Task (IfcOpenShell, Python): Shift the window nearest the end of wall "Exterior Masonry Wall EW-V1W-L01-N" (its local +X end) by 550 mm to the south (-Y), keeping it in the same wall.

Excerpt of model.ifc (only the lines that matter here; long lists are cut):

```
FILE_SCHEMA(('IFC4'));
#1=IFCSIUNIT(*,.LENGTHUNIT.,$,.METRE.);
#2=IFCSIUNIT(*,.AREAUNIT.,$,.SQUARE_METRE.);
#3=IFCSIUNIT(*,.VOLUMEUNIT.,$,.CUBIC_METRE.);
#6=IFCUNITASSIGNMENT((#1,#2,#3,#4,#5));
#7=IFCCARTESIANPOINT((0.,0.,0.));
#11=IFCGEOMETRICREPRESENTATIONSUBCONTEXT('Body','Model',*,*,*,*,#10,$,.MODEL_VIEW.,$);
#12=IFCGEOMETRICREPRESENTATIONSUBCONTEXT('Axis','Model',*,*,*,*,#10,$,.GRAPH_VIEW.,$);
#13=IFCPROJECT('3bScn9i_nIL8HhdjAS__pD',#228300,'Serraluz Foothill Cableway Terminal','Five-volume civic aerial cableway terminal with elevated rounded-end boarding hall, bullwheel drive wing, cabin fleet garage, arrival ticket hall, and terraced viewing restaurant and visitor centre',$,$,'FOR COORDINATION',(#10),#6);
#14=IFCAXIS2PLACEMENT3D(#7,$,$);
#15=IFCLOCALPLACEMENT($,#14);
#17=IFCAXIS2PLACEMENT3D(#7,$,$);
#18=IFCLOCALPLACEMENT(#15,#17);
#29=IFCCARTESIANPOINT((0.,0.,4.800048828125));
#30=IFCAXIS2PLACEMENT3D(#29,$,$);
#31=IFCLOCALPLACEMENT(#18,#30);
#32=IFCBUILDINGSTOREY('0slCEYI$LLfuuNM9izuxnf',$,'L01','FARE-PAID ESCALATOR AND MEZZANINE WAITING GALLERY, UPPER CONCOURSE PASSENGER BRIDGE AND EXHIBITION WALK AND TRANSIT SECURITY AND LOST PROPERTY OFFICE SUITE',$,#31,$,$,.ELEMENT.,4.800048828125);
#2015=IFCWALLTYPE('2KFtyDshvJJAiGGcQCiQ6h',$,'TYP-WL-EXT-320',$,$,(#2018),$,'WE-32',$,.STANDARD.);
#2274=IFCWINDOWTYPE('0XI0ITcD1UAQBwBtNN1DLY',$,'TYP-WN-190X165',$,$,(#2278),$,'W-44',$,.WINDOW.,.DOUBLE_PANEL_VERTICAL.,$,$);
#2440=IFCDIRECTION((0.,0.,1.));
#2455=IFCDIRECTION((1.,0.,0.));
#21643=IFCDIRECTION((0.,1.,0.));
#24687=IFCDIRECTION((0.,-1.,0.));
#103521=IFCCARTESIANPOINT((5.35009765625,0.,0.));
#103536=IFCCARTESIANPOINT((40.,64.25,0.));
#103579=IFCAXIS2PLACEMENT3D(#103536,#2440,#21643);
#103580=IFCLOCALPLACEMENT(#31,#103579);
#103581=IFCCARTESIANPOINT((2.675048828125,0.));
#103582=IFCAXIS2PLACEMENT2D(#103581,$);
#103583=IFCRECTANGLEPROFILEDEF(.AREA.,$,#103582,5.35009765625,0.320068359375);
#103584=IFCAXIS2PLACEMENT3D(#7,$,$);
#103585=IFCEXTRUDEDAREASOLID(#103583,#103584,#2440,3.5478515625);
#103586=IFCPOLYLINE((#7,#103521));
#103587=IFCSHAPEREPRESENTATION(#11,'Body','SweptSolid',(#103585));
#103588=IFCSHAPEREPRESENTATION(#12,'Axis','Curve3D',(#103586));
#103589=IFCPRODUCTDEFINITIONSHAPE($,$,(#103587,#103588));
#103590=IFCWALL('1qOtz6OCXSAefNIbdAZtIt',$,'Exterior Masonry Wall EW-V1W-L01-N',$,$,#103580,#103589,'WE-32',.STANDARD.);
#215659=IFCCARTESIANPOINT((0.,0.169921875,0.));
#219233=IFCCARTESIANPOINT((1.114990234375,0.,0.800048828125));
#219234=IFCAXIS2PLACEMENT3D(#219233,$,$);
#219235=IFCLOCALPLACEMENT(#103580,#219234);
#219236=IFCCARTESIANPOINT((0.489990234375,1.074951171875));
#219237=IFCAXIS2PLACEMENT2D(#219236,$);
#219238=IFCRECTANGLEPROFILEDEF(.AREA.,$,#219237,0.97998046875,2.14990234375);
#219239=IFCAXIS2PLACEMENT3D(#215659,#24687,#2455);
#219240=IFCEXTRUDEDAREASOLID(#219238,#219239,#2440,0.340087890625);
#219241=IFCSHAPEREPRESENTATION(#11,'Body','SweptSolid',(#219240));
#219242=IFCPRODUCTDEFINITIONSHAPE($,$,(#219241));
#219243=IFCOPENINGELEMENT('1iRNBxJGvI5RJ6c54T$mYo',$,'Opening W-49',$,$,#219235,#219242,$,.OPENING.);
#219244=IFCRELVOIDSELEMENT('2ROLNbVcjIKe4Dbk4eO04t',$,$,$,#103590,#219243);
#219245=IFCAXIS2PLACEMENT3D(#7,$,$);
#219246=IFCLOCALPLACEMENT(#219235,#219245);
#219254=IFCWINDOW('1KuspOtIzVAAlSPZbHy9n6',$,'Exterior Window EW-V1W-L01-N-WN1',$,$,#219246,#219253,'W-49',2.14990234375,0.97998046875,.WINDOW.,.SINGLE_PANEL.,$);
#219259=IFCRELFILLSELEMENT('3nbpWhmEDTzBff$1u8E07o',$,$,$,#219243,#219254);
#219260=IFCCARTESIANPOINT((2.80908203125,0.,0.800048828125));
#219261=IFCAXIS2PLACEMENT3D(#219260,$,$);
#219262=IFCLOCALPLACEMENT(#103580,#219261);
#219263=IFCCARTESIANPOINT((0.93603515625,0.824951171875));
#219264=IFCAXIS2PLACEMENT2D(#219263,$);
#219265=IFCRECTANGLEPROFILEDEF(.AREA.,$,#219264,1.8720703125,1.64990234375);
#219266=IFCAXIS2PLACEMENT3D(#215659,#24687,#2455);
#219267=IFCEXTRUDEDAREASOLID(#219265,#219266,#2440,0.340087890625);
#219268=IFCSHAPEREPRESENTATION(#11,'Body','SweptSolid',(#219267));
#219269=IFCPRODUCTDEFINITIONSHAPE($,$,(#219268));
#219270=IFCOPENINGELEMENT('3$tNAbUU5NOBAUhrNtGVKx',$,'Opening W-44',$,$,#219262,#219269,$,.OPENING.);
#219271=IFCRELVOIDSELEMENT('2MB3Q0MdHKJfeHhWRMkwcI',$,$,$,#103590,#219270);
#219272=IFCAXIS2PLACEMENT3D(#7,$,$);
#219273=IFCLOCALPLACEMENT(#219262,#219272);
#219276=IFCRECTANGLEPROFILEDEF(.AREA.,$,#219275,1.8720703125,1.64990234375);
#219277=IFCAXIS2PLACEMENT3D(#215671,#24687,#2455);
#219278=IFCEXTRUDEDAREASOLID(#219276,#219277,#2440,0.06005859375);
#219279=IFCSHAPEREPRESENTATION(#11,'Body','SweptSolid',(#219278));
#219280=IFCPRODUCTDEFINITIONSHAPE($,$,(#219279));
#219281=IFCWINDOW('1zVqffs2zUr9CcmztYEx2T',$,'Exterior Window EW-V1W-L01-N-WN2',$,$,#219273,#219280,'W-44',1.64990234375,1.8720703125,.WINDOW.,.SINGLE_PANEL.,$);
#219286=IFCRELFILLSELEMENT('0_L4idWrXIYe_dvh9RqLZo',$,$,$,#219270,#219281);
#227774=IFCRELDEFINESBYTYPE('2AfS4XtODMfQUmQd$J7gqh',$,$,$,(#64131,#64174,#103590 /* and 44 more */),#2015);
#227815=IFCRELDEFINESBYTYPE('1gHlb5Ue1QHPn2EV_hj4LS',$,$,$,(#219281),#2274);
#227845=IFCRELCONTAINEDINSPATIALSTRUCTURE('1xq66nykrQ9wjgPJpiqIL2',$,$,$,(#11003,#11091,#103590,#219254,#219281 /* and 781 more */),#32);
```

```python
import ifcopenshell
import ifcopenshell.api.geometry
import ifcopenshell.util.placement
import ifcopenshell.util.unit

model = ifcopenshell.open("model.ifc")
unit_scale = ifcopenshell.util.unit.calculate_unit_scale(model)

window = model.by_guid("1zVqffs2zUr9CcmztYEx2T")
opening = window.FillsVoids[0].RelatingOpeningElement
wall = opening.VoidsElements[0].RelatingBuildingElement

wall_matrix = ifcopenshell.util.placement.get_local_placement(wall.ObjectPlacement)
shift = wall_matrix[:3, 0] * -0.55 / unit_scale
before = ifcopenshell.util.placement.get_local_placement(window.ObjectPlacement)[:3, 3].copy()

# The window is placed relative to its opening, so it follows when the opening moves.
matrix = ifcopenshell.util.placement.get_local_placement(opening.ObjectPlacement)
matrix[:3, 3] += shift
ifcopenshell.api.geometry.edit_object_placement(
    model, product=opening, matrix=matrix, is_si=False, should_transform_children=True
)

after = ifcopenshell.util.placement.get_local_placement(window.ObjectPlacement)[:3, 3]
print("window moved by", (after - before).round(3) + 0.0)

model.write("model_v2.ifc")
```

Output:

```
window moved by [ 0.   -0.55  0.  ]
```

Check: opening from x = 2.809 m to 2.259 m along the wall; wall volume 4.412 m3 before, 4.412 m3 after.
